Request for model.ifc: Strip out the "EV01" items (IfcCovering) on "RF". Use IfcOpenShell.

First a look at what the model holds.

```python
import ifcopenshell
import ifcopenshell.util.element

model = ifcopenshell.open("model.ifc")
print(model.schema)
storey = next(s for s in model.by_type("IfcBuildingStorey") if s.Name == "RF")
coverings = [e for e in ifcopenshell.util.element.get_decomposition(storey) if e.is_a("IfcCovering")]
seen = {}
for e in coverings:
    element_type = ifcopenshell.util.element.get_type(e)
    name = element_type.Name if element_type not in (None, e) else None
    seen[name] = seen.get(name, 0) + 1
for name, count in sorted(seen.items(), key=str):
    print(count, "x", name)
```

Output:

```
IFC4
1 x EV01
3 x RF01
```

```python
import ifcopenshell
import ifcopenshell.api.root
import ifcopenshell.util.element

model = ifcopenshell.open("model.ifc")

storey = next(s for s in model.by_type("IfcBuildingStorey") if s.Name == "RF")
coverings = [e for e in ifcopenshell.util.element.get_decomposition(storey) if e.is_a("IfcCovering")]
targets = [e for e in coverings if (t := ifcopenshell.util.element.get_type(e)) not in (None, e) and t.Name == "EV01"]

for e in targets:
    ifcopenshell.api.root.remove_product(model, product=e)
print(len(targets), "removed")

model.write("model_rev.ifc")
```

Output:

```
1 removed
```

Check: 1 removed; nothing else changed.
